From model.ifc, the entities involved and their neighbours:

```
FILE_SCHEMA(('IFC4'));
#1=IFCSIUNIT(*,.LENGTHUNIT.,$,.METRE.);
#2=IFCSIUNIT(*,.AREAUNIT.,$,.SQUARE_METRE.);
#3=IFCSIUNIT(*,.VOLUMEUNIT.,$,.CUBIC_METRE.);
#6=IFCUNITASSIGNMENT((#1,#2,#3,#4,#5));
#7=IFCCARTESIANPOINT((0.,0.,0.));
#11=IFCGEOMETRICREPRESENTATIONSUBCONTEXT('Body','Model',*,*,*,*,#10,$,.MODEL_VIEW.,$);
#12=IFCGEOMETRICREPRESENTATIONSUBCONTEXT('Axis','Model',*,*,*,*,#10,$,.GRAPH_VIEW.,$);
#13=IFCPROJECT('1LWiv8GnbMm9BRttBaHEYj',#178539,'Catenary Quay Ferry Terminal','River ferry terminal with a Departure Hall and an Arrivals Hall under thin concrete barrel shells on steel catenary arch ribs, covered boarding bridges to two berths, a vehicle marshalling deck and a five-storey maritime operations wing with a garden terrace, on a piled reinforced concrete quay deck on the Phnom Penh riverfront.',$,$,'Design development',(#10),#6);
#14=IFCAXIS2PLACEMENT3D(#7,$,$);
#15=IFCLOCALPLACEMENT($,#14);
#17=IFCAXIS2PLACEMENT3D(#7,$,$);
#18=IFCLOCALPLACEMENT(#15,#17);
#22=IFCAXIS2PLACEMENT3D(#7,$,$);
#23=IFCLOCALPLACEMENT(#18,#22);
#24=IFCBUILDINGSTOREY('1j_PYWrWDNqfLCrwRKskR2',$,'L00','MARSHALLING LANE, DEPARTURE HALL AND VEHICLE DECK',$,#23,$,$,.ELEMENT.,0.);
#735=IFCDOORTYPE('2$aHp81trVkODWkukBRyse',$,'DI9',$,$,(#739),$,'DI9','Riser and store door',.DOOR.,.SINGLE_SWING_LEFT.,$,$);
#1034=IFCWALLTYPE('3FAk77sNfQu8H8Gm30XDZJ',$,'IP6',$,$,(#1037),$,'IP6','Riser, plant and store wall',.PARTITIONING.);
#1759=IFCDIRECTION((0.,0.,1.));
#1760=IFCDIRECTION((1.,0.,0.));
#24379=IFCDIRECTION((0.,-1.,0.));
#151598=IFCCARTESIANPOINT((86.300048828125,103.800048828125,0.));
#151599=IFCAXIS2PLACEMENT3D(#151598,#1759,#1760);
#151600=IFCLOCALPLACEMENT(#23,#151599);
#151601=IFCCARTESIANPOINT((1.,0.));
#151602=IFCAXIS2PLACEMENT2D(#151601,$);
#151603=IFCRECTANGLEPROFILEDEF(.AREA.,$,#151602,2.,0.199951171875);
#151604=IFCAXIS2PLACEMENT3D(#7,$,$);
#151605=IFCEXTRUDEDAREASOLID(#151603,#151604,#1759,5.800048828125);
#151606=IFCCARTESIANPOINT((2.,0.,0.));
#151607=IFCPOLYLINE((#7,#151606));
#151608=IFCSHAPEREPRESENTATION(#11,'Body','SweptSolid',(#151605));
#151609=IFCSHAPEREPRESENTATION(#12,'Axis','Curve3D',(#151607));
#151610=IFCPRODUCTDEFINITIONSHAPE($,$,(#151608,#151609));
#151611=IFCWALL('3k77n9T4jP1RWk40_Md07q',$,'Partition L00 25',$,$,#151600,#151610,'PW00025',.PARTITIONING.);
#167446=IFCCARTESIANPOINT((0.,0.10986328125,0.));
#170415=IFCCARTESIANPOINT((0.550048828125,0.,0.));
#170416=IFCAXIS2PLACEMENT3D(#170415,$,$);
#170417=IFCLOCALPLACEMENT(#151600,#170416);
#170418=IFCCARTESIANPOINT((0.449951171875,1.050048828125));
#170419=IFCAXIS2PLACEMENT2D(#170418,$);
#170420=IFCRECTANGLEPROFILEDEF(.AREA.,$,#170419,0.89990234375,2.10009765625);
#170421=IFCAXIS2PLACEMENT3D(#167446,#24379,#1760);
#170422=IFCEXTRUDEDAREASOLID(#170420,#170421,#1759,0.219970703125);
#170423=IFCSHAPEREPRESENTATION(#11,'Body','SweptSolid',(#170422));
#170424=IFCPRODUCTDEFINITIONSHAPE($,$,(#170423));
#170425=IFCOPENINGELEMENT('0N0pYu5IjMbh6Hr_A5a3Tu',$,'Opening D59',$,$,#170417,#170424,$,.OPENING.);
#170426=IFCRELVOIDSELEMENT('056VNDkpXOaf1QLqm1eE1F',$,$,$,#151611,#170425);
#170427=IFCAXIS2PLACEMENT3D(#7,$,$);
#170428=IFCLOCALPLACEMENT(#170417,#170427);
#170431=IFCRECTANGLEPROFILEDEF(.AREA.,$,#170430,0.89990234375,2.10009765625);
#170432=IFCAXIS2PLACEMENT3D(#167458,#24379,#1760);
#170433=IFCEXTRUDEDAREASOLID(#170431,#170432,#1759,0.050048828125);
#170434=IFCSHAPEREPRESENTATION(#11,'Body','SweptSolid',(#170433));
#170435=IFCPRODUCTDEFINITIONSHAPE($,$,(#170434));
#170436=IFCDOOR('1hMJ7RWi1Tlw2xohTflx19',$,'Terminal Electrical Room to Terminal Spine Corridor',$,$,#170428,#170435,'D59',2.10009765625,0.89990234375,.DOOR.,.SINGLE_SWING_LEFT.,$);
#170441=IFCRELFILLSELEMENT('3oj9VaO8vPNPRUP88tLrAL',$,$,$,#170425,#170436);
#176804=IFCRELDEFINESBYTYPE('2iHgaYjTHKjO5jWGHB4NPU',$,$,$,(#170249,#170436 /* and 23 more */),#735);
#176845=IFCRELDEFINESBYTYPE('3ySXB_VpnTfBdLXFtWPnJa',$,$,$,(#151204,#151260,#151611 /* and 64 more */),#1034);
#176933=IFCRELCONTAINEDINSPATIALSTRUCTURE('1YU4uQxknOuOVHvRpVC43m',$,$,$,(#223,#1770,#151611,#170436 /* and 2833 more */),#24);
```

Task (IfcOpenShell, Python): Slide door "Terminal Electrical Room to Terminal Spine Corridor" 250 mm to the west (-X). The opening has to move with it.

```python
import ifcopenshell
import ifcopenshell.api.geometry
import ifcopenshell.util.placement
import ifcopenshell.util.unit

model = ifcopenshell.open("model.ifc")
unit_scale = ifcopenshell.util.unit.calculate_unit_scale(model)

door = model.by_guid("1hMJ7RWi1Tlw2xohTflx19")
opening = door.FillsVoids[0].RelatingOpeningElement
wall = opening.VoidsElements[0].RelatingBuildingElement

wall_matrix = ifcopenshell.util.placement.get_local_placement(wall.ObjectPlacement)
shift = wall_matrix[:3, 0] * -0.25 / unit_scale
before = ifcopenshell.util.placement.get_local_placement(door.ObjectPlacement)[:3, 3].copy()

# The door is placed relative to its opening, so it follows when the opening moves.
matrix = ifcopenshell.util.placement.get_local_placement(opening.ObjectPlacement)
matrix[:3, 3] += shift
ifcopenshell.api.geometry.edit_object_placement(
    model, product=opening, matrix=matrix, is_si=False, should_transform_children=True
)

after = ifcopenshell.util.placement.get_local_placement(door.ObjectPlacement)[:3, 3]
print("door moved by", (after - before).round(3) + 0.0)

model.write("model_v2.ifc")
```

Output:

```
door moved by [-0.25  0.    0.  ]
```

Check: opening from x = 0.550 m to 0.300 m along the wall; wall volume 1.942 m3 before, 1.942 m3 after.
